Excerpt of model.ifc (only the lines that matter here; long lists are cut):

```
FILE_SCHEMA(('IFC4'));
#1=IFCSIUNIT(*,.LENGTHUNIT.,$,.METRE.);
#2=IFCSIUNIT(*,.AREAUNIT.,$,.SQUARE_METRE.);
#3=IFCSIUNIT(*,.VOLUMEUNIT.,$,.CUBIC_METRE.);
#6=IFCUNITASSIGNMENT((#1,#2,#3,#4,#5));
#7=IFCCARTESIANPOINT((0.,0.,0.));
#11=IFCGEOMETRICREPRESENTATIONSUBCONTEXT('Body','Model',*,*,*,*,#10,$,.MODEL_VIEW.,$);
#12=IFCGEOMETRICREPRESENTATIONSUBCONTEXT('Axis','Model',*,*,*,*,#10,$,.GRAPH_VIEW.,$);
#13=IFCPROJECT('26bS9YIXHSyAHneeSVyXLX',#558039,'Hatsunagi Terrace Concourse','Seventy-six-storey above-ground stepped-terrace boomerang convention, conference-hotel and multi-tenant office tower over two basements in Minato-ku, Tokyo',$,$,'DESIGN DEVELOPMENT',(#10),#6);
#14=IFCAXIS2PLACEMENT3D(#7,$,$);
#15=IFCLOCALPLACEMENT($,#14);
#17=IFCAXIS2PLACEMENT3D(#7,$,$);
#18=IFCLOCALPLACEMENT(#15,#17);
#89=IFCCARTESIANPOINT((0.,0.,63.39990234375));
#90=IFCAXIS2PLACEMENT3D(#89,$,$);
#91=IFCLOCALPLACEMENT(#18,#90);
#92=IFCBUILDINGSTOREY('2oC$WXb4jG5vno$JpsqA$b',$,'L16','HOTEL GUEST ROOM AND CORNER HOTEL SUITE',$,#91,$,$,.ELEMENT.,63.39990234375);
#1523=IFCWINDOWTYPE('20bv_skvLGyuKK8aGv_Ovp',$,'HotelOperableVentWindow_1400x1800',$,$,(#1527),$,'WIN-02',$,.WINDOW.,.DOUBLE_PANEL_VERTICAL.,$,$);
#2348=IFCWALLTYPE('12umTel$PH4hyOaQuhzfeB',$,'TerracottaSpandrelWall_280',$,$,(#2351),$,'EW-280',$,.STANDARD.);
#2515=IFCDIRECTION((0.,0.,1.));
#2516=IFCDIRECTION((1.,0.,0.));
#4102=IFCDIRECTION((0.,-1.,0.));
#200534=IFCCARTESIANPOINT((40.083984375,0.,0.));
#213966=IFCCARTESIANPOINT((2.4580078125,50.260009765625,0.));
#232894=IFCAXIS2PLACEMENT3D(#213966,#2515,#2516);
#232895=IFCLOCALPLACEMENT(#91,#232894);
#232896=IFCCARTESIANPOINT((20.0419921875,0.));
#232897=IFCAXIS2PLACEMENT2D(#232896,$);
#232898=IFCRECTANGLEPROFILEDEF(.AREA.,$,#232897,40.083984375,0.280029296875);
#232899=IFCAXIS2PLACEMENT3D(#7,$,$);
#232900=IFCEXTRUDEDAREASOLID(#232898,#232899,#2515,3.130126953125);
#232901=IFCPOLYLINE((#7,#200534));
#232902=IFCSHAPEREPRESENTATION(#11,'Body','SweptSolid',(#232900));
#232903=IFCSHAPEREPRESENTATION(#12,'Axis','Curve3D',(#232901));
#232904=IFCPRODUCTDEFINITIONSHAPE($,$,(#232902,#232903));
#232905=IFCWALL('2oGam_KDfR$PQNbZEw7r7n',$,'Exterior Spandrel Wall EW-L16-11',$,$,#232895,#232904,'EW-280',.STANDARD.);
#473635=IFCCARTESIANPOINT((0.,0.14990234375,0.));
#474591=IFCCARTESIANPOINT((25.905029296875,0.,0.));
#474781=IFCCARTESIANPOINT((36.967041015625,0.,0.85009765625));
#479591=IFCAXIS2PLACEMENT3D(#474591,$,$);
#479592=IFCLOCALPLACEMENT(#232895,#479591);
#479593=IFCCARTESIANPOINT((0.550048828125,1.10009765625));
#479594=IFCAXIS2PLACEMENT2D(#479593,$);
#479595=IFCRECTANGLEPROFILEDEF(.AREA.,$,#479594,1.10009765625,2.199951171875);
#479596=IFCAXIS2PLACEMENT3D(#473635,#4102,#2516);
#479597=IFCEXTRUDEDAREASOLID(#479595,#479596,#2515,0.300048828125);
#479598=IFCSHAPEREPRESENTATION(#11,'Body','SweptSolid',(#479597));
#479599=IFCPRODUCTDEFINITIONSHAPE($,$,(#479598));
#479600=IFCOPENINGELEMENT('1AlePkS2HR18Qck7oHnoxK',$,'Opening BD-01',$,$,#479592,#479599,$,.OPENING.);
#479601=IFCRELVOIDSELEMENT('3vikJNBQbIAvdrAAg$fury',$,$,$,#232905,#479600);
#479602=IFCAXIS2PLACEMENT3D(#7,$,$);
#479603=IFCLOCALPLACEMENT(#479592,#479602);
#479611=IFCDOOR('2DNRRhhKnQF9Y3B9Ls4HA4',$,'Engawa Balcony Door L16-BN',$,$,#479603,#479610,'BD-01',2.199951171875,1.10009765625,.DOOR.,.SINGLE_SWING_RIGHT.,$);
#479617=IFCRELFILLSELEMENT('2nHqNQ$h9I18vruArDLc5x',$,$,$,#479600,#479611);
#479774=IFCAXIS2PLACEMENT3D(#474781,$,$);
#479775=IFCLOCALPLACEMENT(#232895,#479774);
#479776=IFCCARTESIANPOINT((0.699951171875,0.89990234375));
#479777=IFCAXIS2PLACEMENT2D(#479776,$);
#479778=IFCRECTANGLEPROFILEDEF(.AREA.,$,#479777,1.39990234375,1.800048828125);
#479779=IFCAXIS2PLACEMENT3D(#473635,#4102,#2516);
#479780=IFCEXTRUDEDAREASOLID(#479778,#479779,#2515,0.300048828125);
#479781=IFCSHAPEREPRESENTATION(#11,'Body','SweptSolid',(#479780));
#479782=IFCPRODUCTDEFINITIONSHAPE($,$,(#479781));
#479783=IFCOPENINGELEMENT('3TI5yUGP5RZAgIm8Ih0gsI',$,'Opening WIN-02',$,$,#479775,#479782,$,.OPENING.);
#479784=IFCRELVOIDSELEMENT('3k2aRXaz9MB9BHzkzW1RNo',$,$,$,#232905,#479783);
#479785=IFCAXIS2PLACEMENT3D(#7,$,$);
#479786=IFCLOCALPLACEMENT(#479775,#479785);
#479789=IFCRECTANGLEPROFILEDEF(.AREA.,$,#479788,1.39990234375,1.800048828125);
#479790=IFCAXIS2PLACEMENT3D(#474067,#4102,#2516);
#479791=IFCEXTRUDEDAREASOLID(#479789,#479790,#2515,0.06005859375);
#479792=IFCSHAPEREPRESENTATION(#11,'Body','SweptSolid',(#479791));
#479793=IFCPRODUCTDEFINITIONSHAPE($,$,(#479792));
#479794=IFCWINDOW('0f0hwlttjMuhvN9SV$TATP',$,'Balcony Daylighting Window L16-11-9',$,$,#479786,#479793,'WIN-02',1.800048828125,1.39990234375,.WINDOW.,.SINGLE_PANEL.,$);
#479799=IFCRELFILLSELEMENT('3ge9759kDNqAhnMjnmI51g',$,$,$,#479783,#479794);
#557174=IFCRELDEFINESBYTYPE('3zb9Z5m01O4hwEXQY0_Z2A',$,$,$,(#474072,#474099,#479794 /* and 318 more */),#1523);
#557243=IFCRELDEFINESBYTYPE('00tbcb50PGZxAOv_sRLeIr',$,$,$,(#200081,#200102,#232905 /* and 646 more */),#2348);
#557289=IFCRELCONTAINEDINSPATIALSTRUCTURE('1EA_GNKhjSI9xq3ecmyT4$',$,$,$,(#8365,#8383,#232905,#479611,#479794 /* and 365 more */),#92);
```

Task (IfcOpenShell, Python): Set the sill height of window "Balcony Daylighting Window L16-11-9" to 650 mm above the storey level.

```python
import numpy as np
import ifcopenshell
import ifcopenshell.api.geometry
import ifcopenshell.geom
import ifcopenshell.util.element
import ifcopenshell.util.placement
import ifcopenshell.util.shape
import ifcopenshell.util.unit

model = ifcopenshell.open("model.ifc")
unit_scale = ifcopenshell.util.unit.calculate_unit_scale(model)

window = model.by_guid("0f0hwlttjMuhvN9SV$TATP")
opening = window.FillsVoids[0].RelatingOpeningElement
storey = ifcopenshell.util.element.get_container(window, ifc_class="IfcBuildingStorey")
level = ifcopenshell.util.placement.get_local_placement(storey.ObjectPlacement)[2, 3]

# The opening's origin need not be at the sill, so measure its lowest point.
shape = ifcopenshell.geom.create_shape(ifcopenshell.geom.settings(), opening)
bottom = ifcopenshell.util.shape.get_shape_bottom_elevation(shape, shape.geometry) / unit_scale
dz = level + 0.65 - bottom

shift = np.array([0.0, 0.0, dz])
# The window is placed relative to its opening, so it follows when the opening moves.
matrix = ifcopenshell.util.placement.get_local_placement(opening.ObjectPlacement)
matrix[:3, 3] += shift
ifcopenshell.api.geometry.edit_object_placement(
    model, product=opening, matrix=matrix, is_si=False, should_transform_children=True
)

print(f"moved by {dz * unit_scale:+.3f} m")

model.write("model_rev.ifc")
```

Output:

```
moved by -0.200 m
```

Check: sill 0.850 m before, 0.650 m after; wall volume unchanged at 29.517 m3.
